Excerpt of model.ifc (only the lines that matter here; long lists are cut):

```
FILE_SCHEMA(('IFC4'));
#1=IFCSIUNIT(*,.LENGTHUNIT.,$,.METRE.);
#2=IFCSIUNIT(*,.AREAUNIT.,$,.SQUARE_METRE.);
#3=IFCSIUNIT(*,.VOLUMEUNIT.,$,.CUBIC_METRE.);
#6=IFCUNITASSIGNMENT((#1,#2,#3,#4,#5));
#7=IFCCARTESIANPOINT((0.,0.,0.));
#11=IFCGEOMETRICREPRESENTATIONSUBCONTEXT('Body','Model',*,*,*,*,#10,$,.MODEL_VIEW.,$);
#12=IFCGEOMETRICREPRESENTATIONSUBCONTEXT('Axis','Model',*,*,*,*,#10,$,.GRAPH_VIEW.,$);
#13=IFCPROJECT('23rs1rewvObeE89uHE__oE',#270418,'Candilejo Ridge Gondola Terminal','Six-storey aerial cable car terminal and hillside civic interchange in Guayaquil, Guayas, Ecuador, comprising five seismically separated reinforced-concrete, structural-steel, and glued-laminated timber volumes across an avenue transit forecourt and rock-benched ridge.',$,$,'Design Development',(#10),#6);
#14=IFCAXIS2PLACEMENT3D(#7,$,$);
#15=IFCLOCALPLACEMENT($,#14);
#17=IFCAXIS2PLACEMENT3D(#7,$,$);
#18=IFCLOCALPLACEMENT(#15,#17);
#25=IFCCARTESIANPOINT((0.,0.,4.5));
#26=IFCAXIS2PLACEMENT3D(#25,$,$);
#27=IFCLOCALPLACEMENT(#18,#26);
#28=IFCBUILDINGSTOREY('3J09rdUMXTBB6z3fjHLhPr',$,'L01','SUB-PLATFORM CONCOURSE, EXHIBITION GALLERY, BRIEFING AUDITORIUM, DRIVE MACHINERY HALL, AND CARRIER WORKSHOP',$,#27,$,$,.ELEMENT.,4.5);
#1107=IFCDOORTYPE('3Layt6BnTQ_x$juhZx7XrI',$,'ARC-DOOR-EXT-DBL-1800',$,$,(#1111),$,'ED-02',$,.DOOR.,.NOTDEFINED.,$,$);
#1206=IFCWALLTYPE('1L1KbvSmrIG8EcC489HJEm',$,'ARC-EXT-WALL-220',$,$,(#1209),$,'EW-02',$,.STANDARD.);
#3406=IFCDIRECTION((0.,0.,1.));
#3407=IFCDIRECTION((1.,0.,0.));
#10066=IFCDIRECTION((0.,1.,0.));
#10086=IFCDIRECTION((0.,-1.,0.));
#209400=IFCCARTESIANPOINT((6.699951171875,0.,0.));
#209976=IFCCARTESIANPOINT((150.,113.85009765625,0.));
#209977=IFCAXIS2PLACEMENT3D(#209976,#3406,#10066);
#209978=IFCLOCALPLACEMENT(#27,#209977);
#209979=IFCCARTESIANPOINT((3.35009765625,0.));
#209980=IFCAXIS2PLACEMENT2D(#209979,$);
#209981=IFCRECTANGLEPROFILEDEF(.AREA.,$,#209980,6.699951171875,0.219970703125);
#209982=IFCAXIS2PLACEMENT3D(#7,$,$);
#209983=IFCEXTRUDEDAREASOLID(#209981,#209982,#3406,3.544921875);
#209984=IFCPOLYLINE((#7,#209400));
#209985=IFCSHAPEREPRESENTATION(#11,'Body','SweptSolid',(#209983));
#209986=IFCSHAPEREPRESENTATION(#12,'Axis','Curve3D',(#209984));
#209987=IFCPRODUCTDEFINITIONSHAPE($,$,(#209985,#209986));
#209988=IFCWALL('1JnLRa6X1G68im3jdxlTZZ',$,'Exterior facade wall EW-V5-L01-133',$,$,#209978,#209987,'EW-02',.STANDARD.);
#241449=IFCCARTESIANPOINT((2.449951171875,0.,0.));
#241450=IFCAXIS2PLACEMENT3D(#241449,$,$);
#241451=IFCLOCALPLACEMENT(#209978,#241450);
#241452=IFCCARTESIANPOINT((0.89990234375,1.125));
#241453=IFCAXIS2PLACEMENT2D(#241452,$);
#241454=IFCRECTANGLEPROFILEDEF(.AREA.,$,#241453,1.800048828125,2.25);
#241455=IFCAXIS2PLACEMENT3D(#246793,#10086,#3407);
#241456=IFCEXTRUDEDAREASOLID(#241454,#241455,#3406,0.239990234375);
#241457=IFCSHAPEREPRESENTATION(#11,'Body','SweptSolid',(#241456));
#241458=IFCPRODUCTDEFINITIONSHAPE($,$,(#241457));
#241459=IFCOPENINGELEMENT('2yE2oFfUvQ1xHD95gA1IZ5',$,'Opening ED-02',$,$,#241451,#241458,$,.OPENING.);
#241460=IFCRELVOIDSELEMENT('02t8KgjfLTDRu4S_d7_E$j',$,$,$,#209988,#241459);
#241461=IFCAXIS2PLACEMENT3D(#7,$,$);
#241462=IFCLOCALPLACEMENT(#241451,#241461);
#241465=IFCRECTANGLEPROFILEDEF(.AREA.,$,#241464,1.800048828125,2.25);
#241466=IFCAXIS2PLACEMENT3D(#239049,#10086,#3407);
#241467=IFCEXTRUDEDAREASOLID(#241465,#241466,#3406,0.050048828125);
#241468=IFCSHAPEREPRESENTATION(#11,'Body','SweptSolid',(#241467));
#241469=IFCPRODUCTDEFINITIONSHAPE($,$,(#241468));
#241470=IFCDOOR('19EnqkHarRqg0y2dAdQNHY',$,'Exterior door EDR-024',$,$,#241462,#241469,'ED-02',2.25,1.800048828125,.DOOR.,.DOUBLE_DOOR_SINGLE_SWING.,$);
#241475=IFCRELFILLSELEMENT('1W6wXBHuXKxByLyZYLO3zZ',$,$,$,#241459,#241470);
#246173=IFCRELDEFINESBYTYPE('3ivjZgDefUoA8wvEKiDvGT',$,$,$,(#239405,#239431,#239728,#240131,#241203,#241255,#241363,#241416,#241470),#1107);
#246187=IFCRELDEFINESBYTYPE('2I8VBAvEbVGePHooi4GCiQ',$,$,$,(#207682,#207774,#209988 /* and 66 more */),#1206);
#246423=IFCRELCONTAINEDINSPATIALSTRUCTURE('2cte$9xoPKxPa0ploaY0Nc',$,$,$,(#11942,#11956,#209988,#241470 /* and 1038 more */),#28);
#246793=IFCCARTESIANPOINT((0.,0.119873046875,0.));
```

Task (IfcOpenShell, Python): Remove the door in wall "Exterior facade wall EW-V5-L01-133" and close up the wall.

```python
import ifcopenshell
import ifcopenshell.api.feature
import ifcopenshell.api.root
import ifcopenshell.geom
import ifcopenshell.util.shape

model = ifcopenshell.open("model.ifc")
settings = ifcopenshell.geom.settings()


def volume(element):
    """Net volume in cubic metres, openings subtracted."""
    shape = ifcopenshell.geom.create_shape(settings, element)
    return ifcopenshell.util.shape.get_volume(shape.geometry)


door = model.by_guid("19EnqkHarRqg0y2dAdQNHY")
opening = door.FillsVoids[0].RelatingOpeningElement
wall = opening.VoidsElements[0].RelatingBuildingElement
before = volume(wall)

ifcopenshell.api.root.remove_product(model, product=door)
ifcopenshell.api.feature.remove_feature(model, feature=opening)

after = volume(wall)

print(f"wall volume {before:.3f} -> {after:.3f} m3")

model.write("model_rev.ifc")
```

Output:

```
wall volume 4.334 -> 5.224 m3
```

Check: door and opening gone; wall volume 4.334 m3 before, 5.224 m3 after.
